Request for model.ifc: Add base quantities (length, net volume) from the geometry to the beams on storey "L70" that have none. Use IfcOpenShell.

First a look at what the model holds.

```python
import ifcopenshell
import ifcopenshell.util.element
import ifcopenshell.util.unit

model = ifcopenshell.open("model.ifc")
print(model.schema)
for unit_type in ("LENGTHUNIT", "AREAUNIT", "VOLUMEUNIT"):
    print(unit_type, ifcopenshell.util.unit.calculate_unit_scale(model, unit_type))
storey = next(s for s in model.by_type("IfcBuildingStorey") if s.Name == "L70")
beams = [e for e in ifcopenshell.util.element.get_decomposition(storey) if e.is_a("IfcBeam")]
for e in sorted(beams, key=lambda e: e.id()):
    print(e.id(), e.is_a(), e.Name, list(ifcopenshell.util.element.get_psets(e, qtos_only=True)), sep=" | ")
```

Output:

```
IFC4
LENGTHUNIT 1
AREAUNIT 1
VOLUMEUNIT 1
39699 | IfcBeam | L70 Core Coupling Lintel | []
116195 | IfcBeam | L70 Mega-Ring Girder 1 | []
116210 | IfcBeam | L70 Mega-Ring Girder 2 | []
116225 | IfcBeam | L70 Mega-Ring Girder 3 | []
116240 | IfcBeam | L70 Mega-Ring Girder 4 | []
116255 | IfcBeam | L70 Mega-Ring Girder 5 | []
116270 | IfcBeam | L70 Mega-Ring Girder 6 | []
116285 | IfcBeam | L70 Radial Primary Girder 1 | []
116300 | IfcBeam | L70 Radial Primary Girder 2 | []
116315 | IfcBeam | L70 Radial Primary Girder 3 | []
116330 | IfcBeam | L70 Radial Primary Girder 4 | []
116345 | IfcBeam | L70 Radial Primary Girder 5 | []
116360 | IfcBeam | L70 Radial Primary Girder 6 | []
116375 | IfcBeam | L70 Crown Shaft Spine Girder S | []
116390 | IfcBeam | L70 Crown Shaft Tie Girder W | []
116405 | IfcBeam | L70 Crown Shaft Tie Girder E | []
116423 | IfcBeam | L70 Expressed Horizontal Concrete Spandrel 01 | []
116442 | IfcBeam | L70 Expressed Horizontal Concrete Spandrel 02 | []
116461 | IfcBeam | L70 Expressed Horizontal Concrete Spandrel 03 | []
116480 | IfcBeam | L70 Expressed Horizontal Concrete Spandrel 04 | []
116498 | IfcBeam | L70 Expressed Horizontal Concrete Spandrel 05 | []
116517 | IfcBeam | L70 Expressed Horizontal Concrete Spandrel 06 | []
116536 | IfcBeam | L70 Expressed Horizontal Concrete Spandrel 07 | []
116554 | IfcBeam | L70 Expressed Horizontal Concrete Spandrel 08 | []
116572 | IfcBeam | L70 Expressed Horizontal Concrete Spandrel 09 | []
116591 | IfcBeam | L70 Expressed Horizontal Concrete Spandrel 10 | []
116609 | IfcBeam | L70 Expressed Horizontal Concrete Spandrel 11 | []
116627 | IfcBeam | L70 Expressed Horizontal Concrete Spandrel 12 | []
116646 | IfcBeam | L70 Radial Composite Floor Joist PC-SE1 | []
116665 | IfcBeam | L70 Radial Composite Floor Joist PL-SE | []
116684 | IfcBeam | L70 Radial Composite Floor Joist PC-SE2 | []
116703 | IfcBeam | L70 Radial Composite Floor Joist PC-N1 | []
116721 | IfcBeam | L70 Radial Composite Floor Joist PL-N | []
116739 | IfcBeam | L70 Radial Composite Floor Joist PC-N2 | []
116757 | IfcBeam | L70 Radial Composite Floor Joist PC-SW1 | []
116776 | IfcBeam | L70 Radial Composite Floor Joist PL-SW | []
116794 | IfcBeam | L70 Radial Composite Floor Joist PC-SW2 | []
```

```python
import ifcopenshell
import ifcopenshell.api.pset
import ifcopenshell.geom
import ifcopenshell.util.element
import ifcopenshell.util.shape
import ifcopenshell.util.unit

model = ifcopenshell.open("model.ifc")
unit_scale = ifcopenshell.util.unit.calculate_unit_scale(model)
volume_scale = ifcopenshell.util.unit.calculate_unit_scale(model, "VOLUMEUNIT")
settings = ifcopenshell.geom.settings()

storey = next(s for s in model.by_type("IfcBuildingStorey") if s.Name == "L70")
beams = [e for e in ifcopenshell.util.element.get_decomposition(storey) if e.is_a("IfcBeam")]

for e in sorted(beams, key=lambda e: e.id()):
    if ifcopenshell.util.element.get_psets(e, qtos_only=True, should_inherit=False):
        continue
    # Geometry comes back in metres, in the element's own axes.
    shape = ifcopenshell.geom.create_shape(settings, e)
    values = {
        "Length": ifcopenshell.util.shape.get_max_xyz(shape.geometry) / unit_scale,
        "NetVolume": ifcopenshell.util.shape.get_volume(shape.geometry) / volume_scale,
    }
    qto = ifcopenshell.api.pset.add_qto(model, product=e, name="Qto_BeamBaseQuantities")
    ifcopenshell.api.pset.edit_qto(model, qto=qto, properties=values)
    print(e.id(), {k: round(v, 3) for k, v in values.items()})

model.write("model_updated.ifc")
```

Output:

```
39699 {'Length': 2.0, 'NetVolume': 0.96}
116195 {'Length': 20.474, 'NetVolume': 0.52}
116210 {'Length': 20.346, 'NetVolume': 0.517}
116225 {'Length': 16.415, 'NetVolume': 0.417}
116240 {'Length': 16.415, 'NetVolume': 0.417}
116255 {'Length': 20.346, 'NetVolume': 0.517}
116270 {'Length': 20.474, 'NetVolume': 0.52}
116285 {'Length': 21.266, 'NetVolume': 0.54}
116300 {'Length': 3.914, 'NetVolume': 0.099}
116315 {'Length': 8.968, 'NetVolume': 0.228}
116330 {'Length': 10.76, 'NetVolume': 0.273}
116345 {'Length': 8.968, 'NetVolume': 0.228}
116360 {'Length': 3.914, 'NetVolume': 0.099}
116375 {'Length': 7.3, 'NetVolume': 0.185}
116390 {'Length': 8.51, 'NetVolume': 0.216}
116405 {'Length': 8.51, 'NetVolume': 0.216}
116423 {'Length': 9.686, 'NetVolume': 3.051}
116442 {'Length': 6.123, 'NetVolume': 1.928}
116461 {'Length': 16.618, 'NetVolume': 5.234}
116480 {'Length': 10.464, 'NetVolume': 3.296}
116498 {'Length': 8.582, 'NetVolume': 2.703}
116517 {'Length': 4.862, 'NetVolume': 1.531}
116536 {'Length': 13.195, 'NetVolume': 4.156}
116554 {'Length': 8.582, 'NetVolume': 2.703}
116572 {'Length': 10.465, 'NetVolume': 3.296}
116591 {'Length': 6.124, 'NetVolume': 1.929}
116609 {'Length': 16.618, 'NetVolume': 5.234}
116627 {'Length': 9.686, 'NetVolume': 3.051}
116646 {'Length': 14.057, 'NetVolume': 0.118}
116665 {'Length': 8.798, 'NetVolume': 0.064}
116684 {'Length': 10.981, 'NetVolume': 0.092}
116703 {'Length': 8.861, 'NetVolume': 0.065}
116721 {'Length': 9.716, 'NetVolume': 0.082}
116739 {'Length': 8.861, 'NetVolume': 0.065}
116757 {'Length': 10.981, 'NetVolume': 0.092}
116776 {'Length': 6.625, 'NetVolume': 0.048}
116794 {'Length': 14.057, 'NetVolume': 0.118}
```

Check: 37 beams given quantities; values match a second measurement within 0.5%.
